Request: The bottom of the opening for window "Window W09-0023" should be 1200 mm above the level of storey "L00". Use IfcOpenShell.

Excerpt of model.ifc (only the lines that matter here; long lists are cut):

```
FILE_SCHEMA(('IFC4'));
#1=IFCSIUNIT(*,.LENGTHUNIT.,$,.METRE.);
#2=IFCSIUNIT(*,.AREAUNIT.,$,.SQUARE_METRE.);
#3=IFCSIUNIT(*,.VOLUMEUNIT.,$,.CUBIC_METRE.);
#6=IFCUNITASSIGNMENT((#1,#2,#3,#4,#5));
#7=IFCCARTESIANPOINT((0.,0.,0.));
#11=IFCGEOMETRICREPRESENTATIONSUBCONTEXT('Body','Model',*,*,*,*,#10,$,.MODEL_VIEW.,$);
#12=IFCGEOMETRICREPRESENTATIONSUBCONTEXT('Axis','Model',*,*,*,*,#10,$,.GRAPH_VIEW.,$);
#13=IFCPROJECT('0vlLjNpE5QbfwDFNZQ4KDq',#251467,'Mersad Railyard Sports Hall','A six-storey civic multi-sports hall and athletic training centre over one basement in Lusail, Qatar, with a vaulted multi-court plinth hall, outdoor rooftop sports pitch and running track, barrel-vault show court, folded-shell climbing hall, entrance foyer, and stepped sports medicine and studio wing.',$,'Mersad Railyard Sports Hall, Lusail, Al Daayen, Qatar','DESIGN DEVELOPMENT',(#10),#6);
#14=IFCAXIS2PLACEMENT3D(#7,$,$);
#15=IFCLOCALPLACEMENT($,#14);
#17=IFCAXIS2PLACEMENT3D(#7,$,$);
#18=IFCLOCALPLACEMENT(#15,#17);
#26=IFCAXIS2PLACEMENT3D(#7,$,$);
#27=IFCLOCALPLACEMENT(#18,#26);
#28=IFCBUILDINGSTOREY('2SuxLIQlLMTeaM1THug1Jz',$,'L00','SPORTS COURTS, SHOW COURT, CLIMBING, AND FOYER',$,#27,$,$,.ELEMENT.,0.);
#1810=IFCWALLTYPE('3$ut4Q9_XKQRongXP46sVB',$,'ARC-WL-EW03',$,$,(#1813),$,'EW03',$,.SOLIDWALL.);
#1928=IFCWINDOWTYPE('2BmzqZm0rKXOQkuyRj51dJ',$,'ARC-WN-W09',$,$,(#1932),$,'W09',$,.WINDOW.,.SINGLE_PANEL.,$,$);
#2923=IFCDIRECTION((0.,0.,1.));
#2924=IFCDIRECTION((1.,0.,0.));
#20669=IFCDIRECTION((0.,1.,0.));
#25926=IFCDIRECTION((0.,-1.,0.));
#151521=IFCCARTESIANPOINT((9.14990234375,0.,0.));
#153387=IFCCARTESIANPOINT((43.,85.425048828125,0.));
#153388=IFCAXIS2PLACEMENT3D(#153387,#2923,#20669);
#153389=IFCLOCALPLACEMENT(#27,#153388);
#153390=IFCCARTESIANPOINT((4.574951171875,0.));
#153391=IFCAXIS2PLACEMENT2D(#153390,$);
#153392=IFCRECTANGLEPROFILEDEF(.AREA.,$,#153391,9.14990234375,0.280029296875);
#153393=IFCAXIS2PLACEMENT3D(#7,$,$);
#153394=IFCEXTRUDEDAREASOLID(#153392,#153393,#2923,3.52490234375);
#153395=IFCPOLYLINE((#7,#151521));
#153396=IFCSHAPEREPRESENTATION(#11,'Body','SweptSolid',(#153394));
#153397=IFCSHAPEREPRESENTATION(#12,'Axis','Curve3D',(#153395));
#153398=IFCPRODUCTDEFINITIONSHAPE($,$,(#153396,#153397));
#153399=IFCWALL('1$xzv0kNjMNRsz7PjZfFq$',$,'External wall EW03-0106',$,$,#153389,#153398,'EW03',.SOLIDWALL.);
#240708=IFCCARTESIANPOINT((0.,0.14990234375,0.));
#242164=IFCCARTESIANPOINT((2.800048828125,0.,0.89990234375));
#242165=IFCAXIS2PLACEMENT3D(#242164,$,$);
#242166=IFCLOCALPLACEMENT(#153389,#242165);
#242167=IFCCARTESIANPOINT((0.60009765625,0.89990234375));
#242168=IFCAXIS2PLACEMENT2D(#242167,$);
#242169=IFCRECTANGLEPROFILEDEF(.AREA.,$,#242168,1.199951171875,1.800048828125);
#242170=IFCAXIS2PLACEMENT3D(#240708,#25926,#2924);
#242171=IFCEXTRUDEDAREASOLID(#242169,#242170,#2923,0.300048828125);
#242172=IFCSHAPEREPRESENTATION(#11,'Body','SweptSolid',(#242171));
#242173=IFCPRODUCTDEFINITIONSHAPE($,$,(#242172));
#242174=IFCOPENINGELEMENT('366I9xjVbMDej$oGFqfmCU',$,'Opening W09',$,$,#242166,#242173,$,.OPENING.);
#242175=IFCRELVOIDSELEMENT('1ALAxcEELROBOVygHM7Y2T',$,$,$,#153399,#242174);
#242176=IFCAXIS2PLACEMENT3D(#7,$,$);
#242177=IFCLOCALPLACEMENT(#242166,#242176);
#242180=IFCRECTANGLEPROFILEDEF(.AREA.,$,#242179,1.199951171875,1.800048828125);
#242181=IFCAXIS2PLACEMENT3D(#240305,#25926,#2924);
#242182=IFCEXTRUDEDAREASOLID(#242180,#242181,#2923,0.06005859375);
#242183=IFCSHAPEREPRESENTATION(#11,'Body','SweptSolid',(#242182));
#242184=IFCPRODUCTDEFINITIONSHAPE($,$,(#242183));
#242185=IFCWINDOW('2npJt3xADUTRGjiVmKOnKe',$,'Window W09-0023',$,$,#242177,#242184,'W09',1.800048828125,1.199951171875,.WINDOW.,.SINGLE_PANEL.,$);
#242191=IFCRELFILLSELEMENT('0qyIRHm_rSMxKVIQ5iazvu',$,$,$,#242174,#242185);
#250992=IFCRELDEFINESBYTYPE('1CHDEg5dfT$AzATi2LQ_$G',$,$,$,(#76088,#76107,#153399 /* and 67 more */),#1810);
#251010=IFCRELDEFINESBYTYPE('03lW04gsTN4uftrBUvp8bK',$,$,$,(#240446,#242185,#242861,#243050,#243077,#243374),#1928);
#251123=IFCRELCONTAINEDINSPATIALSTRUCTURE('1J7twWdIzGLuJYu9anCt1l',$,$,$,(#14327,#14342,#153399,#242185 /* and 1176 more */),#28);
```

```python
import numpy as np
import ifcopenshell
import ifcopenshell.api.geometry
import ifcopenshell.geom
import ifcopenshell.util.element
import ifcopenshell.util.placement
import ifcopenshell.util.shape
import ifcopenshell.util.unit

model = ifcopenshell.open("model.ifc")
unit_scale = ifcopenshell.util.unit.calculate_unit_scale(model)

window = model.by_guid("2npJt3xADUTRGjiVmKOnKe")
opening = window.FillsVoids[0].RelatingOpeningElement
storey = ifcopenshell.util.element.get_container(window, ifc_class="IfcBuildingStorey")
level = ifcopenshell.util.placement.get_local_placement(storey.ObjectPlacement)[2, 3]

# The opening's origin need not be at the sill, so measure its lowest point.
shape = ifcopenshell.geom.create_shape(ifcopenshell.geom.settings(), opening)
bottom = ifcopenshell.util.shape.get_shape_bottom_elevation(shape, shape.geometry) / unit_scale
dz = level + 1.2 / unit_scale - bottom

shift = np.array([0.0, 0.0, dz])
# The window is placed relative to its opening, so it follows when the opening moves.
matrix = ifcopenshell.util.placement.get_local_placement(opening.ObjectPlacement)
matrix[:3, 3] += shift
ifcopenshell.api.geometry.edit_object_placement(
    model, product=opening, matrix=matrix, is_si=False, should_transform_children=True
)

print(f"moved by {dz * unit_scale:+.3f} m")

model.write("model_v2.ifc")
```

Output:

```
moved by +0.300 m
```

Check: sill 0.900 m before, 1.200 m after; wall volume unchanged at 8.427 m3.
